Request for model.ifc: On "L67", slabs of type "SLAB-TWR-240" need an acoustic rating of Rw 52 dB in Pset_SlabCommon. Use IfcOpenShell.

First a look at what the model holds.

```python
import ifcopenshell
import ifcopenshell.util.element

model = ifcopenshell.open("model.ifc")
print(model.schema)
storey = next(s for s in model.by_type("IfcBuildingStorey") if s.Name == "L67")
slabs = [e for e in ifcopenshell.util.element.get_decomposition(storey) if e.is_a("IfcSlab")]
seen = {}
for e in slabs:
    element_type = ifcopenshell.util.element.get_type(e)
    key = (element_type.Name if element_type != e and element_type else None, ifcopenshell.util.element.get_pset(e, "Pset_SlabCommon", "AcousticRating"))
    seen[key] = seen.get(key, 0) + 1
for (name, value), count in sorted(seen.items(), key=str):
    print(count, "x", name, "|", value)
```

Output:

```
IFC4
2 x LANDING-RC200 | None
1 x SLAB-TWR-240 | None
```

```python
import ifcopenshell
import ifcopenshell.api.pset
import ifcopenshell.util.element

model = ifcopenshell.open("model.ifc")

storey = next(s for s in model.by_type("IfcBuildingStorey") if s.Name == "L67")
slabs = [e for e in ifcopenshell.util.element.get_decomposition(storey) if e.is_a("IfcSlab")]

count = 0
for e in slabs:
    element_type = ifcopenshell.util.element.get_type(e)
    if element_type in (None, e) or element_type.Name != "SLAB-TWR-240":
        continue
    # add_pset returns the element's existing set when there is one.
    pset = ifcopenshell.api.pset.add_pset(model, product=e, name="Pset_SlabCommon")
    ifcopenshell.api.pset.edit_pset(model, pset=pset, properties={"AcousticRating": "Rw 52 dB"})
    count += 1

print(count, "slabs updated")

model.write("model_rev.ifc")
```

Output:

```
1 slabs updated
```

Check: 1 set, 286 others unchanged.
